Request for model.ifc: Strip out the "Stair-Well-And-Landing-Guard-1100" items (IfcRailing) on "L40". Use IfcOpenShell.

First a look at what the model holds.

```python
import ifcopenshell
import ifcopenshell.util.element

model = ifcopenshell.open("model.ifc")
print(model.schema)
storey = next(s for s in model.by_type("IfcBuildingStorey") if s.Name == "L40")
railings = [e for e in ifcopenshell.util.element.get_decomposition(storey) if e.is_a("IfcRailing")]
seen = {}
for e in railings:
    element_type = ifcopenshell.util.element.get_type(e)
    name = element_type.Name if element_type not in (None, e) else None
    seen[name] = seen.get(name, 0) + 1
for name, count in sorted(seen.items(), key=str):
    print(count, "x", name)
```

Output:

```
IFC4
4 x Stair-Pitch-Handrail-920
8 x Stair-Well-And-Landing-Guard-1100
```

```python
import ifcopenshell
import ifcopenshell.api.root
import ifcopenshell.util.element

model = ifcopenshell.open("model.ifc")

storey = next(s for s in model.by_type("IfcBuildingStorey") if s.Name == "L40")
railings = [e for e in ifcopenshell.util.element.get_decomposition(storey) if e.is_a("IfcRailing")]
targets = [e for e in railings if (t := ifcopenshell.util.element.get_type(e)) not in (None, e) and t.Name == "Stair-Well-And-Landing-Guard-1100"]

for e in targets:
    ifcopenshell.api.root.remove_product(model, product=e)
print(len(targets), "removed")

model.write("model-out.ifc")
```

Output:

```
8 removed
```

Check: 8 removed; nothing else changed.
